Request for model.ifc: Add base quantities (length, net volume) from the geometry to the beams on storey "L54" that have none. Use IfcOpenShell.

First a look at what the model holds.

```python
import ifcopenshell
import ifcopenshell.util.element
import ifcopenshell.util.unit

model = ifcopenshell.open("model.ifc")
print(model.schema)
for unit_type in ("LENGTHUNIT", "AREAUNIT", "VOLUMEUNIT"):
    print(unit_type, ifcopenshell.util.unit.calculate_unit_scale(model, unit_type))
storey = next(s for s in model.by_type("IfcBuildingStorey") if s.Name == "L54")
beams = [e for e in ifcopenshell.util.element.get_decomposition(storey) if e.is_a("IfcBeam")]
for e in sorted(beams, key=lambda e: e.id()):
    print(e.id(), e.is_a(), e.Name, list(ifcopenshell.util.element.get_psets(e, qtos_only=True)), sep=" | ")
```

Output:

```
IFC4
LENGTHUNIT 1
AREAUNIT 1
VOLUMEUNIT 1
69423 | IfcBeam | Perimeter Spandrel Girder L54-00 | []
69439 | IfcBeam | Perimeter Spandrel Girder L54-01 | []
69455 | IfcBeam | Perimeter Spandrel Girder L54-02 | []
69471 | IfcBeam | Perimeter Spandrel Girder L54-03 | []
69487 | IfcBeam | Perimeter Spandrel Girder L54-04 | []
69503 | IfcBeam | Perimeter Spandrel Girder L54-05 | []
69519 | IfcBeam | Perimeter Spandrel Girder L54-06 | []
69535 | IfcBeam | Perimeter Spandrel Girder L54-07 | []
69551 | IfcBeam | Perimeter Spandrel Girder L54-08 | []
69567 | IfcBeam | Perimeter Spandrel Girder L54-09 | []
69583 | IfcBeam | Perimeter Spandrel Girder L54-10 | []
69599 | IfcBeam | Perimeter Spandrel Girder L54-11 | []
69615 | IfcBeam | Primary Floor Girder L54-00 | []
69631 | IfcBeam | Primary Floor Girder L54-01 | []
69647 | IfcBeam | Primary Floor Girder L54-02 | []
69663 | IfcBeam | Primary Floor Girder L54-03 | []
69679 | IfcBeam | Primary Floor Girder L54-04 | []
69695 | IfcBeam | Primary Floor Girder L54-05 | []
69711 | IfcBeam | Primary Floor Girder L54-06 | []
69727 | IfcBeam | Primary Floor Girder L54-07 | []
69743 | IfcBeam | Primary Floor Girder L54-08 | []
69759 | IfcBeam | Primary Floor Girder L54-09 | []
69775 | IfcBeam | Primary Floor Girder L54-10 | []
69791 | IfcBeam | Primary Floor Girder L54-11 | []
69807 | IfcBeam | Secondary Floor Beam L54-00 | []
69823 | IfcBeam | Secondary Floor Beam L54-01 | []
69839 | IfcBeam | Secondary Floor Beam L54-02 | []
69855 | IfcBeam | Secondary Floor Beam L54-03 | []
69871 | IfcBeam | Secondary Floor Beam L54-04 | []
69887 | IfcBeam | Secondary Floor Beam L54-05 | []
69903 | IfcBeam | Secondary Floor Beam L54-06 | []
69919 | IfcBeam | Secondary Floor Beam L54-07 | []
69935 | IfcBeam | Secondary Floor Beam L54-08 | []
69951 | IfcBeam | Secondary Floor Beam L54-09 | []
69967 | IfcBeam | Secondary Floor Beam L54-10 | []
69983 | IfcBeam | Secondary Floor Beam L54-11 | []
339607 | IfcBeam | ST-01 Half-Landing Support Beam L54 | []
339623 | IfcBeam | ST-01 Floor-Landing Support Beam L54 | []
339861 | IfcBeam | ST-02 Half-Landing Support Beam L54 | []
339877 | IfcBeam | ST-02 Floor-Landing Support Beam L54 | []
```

```python
import ifcopenshell
import ifcopenshell.api.pset
import ifcopenshell.geom
import ifcopenshell.util.element
import ifcopenshell.util.shape
import ifcopenshell.util.unit

model = ifcopenshell.open("model.ifc")
unit_scale = ifcopenshell.util.unit.calculate_unit_scale(model)
volume_scale = ifcopenshell.util.unit.calculate_unit_scale(model, "VOLUMEUNIT")
settings = ifcopenshell.geom.settings()

storey = next(s for s in model.by_type("IfcBuildingStorey") if s.Name == "L54")
beams = [e for e in ifcopenshell.util.element.get_decomposition(storey) if e.is_a("IfcBeam")]

for e in sorted(beams, key=lambda e: e.id()):
    if ifcopenshell.util.element.get_psets(e, qtos_only=True, should_inherit=False):
        continue
    # Geometry comes back in metres, in the element's own axes.
    shape = ifcopenshell.geom.create_shape(settings, e)
    values = {
        "Length": ifcopenshell.util.shape.get_max_xyz(shape.geometry) / unit_scale,
        "NetVolume": ifcopenshell.util.shape.get_volume(shape.geometry) / volume_scale,
    }
    qto = ifcopenshell.api.pset.add_qto(model, product=e, name="Qto_BeamBaseQuantities")
    ifcopenshell.api.pset.edit_qto(model, qto=qto, properties=values)
    print(e.id(), {k: round(v, 3) for k, v in values.items()})

model.write("model_v2.ifc")
```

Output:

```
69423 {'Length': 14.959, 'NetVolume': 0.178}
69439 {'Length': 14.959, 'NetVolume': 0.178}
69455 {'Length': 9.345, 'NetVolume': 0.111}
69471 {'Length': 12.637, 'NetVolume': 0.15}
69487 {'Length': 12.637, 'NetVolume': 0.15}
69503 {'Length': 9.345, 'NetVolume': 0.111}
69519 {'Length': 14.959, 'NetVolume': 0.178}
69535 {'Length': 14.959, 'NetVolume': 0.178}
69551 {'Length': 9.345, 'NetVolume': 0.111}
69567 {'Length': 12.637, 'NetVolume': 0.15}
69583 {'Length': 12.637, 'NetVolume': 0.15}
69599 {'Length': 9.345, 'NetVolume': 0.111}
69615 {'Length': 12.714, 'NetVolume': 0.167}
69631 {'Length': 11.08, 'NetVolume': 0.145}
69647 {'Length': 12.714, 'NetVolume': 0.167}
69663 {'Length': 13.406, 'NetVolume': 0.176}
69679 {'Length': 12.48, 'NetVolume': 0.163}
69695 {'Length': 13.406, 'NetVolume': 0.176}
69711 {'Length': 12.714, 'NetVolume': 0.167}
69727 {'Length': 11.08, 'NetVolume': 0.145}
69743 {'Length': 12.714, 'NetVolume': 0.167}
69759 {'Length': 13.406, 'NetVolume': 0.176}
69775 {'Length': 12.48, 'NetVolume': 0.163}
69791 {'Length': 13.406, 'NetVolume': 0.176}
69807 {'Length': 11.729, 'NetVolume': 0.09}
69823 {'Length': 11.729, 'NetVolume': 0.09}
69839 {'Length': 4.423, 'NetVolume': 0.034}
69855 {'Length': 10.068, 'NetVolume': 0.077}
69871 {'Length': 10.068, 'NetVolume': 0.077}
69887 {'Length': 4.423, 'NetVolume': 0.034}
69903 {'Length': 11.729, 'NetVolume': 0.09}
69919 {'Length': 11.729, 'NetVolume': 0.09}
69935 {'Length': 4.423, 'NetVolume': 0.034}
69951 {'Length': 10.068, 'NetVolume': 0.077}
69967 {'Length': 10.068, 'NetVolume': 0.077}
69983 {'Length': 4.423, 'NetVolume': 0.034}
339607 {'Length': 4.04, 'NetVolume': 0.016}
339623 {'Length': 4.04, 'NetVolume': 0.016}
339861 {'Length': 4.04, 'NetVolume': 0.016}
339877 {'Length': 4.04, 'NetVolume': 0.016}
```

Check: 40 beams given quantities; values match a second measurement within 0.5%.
